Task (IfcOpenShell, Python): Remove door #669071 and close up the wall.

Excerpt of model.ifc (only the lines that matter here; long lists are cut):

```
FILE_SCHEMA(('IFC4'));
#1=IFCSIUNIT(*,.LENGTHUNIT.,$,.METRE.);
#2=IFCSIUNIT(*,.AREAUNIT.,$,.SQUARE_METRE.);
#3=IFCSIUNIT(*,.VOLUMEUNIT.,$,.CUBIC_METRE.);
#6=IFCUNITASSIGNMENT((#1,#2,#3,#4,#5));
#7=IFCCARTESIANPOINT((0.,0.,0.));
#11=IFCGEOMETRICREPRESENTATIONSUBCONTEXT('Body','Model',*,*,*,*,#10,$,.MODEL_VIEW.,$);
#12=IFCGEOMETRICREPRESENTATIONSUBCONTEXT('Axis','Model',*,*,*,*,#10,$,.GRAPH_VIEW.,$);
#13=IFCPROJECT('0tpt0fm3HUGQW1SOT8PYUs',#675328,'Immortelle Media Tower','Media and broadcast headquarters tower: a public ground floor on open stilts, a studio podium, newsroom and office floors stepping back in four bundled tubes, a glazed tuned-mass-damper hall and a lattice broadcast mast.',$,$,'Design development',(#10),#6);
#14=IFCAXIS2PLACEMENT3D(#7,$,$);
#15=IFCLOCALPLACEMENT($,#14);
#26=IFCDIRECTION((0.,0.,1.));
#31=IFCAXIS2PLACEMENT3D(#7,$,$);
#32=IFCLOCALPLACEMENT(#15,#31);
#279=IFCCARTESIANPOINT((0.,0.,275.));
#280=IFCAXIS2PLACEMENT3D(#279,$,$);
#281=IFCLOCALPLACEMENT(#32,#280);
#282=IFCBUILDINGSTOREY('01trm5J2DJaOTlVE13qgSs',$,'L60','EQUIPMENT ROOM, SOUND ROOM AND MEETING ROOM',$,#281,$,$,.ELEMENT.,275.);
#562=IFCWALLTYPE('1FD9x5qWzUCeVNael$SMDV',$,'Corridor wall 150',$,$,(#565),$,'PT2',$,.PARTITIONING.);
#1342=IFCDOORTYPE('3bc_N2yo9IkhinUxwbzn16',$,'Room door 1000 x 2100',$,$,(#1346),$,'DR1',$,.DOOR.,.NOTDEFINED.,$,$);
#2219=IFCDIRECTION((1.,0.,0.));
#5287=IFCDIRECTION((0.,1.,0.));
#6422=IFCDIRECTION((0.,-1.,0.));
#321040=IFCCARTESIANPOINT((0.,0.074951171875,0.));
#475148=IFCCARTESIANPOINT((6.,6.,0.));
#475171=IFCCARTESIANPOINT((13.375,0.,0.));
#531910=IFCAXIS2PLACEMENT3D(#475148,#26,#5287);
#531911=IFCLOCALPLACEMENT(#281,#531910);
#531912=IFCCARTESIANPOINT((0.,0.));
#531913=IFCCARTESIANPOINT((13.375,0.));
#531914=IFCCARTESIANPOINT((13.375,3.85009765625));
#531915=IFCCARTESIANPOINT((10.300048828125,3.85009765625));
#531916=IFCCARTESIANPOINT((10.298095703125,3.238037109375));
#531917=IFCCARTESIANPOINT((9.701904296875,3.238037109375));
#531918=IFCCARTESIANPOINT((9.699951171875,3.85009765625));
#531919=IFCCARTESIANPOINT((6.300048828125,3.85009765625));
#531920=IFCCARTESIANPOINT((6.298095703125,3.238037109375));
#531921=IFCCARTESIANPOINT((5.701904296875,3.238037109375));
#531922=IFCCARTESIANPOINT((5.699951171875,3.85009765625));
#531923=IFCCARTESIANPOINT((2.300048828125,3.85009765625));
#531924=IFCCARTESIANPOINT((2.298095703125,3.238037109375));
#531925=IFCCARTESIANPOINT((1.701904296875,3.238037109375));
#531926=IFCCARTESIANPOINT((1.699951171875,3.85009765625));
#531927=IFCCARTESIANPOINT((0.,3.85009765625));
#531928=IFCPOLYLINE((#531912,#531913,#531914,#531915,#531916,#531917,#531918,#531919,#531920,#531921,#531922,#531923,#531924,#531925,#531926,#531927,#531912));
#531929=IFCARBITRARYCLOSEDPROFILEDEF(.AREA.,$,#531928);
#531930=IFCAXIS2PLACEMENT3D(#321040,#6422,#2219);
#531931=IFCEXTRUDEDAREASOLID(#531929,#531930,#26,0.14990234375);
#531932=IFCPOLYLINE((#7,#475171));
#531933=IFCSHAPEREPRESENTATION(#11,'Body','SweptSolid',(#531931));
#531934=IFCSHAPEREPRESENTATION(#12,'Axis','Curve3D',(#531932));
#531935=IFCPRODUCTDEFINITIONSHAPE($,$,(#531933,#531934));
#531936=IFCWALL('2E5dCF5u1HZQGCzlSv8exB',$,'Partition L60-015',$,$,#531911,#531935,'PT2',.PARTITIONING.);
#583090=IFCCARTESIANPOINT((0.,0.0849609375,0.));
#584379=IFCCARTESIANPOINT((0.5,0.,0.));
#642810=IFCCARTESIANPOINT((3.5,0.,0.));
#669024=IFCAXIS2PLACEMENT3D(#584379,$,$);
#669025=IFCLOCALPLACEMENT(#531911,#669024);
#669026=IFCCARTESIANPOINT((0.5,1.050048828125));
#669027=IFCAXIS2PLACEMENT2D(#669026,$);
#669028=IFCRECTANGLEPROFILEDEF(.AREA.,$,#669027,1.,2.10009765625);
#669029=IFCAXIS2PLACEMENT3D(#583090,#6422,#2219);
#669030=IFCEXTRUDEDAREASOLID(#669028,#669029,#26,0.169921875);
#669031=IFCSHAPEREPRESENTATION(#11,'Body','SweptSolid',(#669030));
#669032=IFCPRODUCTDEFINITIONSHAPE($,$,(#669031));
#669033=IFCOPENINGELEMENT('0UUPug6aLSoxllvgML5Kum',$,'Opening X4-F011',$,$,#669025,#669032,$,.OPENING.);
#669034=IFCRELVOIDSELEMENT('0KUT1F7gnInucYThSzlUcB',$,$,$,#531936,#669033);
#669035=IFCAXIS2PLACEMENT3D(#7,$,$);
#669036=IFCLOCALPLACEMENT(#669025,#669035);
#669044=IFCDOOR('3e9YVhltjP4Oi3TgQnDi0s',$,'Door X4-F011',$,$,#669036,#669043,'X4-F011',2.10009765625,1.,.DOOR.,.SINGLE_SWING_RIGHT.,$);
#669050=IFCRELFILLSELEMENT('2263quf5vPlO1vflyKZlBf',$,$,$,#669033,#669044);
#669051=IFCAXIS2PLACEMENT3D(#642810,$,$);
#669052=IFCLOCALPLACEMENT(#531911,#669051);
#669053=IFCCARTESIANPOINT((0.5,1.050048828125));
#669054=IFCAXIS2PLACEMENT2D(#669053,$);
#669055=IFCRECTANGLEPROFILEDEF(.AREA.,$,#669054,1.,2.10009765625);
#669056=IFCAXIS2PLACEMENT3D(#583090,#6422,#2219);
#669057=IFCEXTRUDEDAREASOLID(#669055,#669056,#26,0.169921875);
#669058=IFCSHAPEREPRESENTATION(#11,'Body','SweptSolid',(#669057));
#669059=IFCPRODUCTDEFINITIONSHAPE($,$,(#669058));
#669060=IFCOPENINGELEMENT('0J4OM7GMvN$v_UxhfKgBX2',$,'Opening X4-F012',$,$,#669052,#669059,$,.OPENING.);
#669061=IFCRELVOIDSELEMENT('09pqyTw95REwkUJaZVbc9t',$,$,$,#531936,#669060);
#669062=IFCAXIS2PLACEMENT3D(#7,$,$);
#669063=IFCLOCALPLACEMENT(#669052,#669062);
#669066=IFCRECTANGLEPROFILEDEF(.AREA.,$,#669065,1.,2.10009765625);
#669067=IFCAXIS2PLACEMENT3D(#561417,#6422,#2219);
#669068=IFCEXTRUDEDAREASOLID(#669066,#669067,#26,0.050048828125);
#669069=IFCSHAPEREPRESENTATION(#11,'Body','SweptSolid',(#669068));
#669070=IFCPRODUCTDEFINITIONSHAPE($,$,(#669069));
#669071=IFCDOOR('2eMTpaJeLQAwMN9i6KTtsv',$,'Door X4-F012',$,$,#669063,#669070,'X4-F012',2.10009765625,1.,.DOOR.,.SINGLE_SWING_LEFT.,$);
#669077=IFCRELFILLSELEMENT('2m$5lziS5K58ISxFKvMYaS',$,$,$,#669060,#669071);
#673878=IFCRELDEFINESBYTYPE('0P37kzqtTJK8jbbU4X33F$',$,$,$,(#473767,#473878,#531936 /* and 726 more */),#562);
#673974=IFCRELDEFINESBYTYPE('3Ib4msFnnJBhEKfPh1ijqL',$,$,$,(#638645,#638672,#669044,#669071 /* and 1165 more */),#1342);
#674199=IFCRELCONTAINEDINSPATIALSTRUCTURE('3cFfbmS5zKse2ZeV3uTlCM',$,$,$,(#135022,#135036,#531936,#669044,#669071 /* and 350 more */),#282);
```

```python
import ifcopenshell
import ifcopenshell.api.feature
import ifcopenshell.api.root
import ifcopenshell.geom
import ifcopenshell.util.shape

model = ifcopenshell.open("model.ifc")
settings = ifcopenshell.geom.settings()


def volume(element):
    """Net volume in cubic metres, openings subtracted."""
    shape = ifcopenshell.geom.create_shape(settings, element)
    return ifcopenshell.util.shape.get_volume(shape.geometry)


door = model.by_guid("2eMTpaJeLQAwMN9i6KTtsv")
opening = door.FillsVoids[0].RelatingOpeningElement
wall = opening.VoidsElements[0].RelatingBuildingElement
before = volume(wall)

ifcopenshell.api.root.remove_product(model, product=door)
ifcopenshell.api.feature.remove_feature(model, feature=opening)

after = volume(wall)

print(f"wall volume {before:.3f} -> {after:.3f} m3")

model.write("model_v2.ifc")
```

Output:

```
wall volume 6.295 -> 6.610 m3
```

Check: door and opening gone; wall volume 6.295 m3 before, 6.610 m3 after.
